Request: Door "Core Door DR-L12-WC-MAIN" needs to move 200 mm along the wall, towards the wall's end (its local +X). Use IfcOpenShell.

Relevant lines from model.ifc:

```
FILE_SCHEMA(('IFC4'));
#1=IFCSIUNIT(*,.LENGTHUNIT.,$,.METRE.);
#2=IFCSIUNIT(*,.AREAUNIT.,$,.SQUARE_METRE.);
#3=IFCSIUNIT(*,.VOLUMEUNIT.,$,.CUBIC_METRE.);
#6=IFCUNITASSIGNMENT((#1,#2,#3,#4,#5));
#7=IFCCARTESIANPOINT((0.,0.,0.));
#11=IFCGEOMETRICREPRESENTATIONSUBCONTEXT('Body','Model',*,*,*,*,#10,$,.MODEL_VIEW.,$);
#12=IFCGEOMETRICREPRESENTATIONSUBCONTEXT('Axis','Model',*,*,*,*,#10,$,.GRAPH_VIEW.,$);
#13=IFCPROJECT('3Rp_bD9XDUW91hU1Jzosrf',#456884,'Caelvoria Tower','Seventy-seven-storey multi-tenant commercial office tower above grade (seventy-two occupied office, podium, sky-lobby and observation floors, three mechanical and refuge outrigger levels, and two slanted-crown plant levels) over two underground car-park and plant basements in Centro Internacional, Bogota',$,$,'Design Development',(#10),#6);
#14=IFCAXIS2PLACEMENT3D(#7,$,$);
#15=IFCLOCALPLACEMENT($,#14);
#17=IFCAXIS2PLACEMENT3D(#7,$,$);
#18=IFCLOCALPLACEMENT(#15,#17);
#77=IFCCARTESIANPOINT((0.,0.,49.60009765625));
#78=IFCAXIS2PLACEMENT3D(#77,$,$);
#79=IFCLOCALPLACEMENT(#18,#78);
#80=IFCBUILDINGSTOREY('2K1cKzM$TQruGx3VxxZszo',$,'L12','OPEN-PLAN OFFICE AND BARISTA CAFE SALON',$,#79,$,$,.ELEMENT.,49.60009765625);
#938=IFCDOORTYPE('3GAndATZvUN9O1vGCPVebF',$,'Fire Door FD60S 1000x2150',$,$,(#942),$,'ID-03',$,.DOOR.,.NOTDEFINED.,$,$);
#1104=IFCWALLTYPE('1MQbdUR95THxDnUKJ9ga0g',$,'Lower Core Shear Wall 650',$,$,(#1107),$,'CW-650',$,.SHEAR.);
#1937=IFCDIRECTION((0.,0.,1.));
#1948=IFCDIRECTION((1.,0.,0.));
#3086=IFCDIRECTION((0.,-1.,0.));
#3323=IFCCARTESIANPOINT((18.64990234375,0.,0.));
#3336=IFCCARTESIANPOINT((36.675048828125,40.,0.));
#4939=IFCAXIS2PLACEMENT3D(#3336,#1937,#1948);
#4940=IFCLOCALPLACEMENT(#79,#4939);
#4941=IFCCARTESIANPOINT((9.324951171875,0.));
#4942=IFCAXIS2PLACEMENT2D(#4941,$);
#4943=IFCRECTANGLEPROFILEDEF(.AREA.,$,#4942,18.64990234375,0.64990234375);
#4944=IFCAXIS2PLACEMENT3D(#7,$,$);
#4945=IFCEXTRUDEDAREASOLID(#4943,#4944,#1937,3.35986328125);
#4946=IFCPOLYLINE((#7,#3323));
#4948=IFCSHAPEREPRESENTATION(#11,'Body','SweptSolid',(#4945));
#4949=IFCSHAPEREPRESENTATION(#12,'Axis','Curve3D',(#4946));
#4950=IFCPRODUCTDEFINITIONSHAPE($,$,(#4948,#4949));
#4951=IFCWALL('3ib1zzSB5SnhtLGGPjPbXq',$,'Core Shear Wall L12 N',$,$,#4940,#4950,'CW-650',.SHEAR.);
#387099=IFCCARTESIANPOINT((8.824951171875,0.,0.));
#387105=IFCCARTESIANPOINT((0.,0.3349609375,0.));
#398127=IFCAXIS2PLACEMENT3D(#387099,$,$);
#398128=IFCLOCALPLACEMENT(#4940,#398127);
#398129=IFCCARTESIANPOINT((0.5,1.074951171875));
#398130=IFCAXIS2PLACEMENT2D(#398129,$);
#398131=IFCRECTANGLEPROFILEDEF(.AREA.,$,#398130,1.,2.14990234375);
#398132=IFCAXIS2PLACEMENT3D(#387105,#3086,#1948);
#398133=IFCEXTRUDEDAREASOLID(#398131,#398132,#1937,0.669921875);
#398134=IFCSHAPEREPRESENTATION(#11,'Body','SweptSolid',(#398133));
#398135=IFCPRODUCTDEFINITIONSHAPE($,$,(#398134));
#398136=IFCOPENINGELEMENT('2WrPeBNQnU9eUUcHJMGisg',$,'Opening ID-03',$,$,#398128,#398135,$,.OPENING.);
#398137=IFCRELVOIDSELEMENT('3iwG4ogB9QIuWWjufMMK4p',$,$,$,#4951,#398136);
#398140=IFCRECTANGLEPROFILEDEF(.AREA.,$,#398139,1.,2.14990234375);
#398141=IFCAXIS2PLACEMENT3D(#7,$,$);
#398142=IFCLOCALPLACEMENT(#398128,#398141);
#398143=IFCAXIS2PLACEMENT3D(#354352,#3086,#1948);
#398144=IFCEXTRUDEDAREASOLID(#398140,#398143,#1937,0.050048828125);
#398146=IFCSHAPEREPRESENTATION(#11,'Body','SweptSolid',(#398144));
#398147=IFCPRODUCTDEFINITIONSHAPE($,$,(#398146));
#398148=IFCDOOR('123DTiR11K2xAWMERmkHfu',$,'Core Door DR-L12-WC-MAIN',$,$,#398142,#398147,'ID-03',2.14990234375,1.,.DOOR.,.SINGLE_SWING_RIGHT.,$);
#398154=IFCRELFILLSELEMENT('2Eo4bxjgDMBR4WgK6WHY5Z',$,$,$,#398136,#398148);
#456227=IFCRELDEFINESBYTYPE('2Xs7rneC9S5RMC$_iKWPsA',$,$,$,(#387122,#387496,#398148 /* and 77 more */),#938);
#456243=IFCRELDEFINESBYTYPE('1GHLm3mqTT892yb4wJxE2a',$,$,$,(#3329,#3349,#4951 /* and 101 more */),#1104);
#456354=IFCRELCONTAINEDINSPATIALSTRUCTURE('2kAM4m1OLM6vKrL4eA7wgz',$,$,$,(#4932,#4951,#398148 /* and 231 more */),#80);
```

```python
import ifcopenshell
import ifcopenshell.api.geometry
import ifcopenshell.util.placement
import ifcopenshell.util.unit

model = ifcopenshell.open("model.ifc")
unit_scale = ifcopenshell.util.unit.calculate_unit_scale(model)

door = model.by_guid("123DTiR11K2xAWMERmkHfu")
opening = door.FillsVoids[0].RelatingOpeningElement
wall = opening.VoidsElements[0].RelatingBuildingElement

wall_matrix = ifcopenshell.util.placement.get_local_placement(wall.ObjectPlacement)
shift = wall_matrix[:3, 0] * 0.2 / unit_scale
before = ifcopenshell.util.placement.get_local_placement(door.ObjectPlacement)[:3, 3].copy()

# The door is placed relative to its opening, so it follows when the opening moves.
matrix = ifcopenshell.util.placement.get_local_placement(opening.ObjectPlacement)
matrix[:3, 3] += shift
ifcopenshell.api.geometry.edit_object_placement(
    model, product=opening, matrix=matrix, is_si=False, should_transform_children=True
)

after = ifcopenshell.util.placement.get_local_placement(door.ObjectPlacement)[:3, 3]
print("door moved by", (after - before).round(3) + 0.0)

model.write("model_rev.ifc")
```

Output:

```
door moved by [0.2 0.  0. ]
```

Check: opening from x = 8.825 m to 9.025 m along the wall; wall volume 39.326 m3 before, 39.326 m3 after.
